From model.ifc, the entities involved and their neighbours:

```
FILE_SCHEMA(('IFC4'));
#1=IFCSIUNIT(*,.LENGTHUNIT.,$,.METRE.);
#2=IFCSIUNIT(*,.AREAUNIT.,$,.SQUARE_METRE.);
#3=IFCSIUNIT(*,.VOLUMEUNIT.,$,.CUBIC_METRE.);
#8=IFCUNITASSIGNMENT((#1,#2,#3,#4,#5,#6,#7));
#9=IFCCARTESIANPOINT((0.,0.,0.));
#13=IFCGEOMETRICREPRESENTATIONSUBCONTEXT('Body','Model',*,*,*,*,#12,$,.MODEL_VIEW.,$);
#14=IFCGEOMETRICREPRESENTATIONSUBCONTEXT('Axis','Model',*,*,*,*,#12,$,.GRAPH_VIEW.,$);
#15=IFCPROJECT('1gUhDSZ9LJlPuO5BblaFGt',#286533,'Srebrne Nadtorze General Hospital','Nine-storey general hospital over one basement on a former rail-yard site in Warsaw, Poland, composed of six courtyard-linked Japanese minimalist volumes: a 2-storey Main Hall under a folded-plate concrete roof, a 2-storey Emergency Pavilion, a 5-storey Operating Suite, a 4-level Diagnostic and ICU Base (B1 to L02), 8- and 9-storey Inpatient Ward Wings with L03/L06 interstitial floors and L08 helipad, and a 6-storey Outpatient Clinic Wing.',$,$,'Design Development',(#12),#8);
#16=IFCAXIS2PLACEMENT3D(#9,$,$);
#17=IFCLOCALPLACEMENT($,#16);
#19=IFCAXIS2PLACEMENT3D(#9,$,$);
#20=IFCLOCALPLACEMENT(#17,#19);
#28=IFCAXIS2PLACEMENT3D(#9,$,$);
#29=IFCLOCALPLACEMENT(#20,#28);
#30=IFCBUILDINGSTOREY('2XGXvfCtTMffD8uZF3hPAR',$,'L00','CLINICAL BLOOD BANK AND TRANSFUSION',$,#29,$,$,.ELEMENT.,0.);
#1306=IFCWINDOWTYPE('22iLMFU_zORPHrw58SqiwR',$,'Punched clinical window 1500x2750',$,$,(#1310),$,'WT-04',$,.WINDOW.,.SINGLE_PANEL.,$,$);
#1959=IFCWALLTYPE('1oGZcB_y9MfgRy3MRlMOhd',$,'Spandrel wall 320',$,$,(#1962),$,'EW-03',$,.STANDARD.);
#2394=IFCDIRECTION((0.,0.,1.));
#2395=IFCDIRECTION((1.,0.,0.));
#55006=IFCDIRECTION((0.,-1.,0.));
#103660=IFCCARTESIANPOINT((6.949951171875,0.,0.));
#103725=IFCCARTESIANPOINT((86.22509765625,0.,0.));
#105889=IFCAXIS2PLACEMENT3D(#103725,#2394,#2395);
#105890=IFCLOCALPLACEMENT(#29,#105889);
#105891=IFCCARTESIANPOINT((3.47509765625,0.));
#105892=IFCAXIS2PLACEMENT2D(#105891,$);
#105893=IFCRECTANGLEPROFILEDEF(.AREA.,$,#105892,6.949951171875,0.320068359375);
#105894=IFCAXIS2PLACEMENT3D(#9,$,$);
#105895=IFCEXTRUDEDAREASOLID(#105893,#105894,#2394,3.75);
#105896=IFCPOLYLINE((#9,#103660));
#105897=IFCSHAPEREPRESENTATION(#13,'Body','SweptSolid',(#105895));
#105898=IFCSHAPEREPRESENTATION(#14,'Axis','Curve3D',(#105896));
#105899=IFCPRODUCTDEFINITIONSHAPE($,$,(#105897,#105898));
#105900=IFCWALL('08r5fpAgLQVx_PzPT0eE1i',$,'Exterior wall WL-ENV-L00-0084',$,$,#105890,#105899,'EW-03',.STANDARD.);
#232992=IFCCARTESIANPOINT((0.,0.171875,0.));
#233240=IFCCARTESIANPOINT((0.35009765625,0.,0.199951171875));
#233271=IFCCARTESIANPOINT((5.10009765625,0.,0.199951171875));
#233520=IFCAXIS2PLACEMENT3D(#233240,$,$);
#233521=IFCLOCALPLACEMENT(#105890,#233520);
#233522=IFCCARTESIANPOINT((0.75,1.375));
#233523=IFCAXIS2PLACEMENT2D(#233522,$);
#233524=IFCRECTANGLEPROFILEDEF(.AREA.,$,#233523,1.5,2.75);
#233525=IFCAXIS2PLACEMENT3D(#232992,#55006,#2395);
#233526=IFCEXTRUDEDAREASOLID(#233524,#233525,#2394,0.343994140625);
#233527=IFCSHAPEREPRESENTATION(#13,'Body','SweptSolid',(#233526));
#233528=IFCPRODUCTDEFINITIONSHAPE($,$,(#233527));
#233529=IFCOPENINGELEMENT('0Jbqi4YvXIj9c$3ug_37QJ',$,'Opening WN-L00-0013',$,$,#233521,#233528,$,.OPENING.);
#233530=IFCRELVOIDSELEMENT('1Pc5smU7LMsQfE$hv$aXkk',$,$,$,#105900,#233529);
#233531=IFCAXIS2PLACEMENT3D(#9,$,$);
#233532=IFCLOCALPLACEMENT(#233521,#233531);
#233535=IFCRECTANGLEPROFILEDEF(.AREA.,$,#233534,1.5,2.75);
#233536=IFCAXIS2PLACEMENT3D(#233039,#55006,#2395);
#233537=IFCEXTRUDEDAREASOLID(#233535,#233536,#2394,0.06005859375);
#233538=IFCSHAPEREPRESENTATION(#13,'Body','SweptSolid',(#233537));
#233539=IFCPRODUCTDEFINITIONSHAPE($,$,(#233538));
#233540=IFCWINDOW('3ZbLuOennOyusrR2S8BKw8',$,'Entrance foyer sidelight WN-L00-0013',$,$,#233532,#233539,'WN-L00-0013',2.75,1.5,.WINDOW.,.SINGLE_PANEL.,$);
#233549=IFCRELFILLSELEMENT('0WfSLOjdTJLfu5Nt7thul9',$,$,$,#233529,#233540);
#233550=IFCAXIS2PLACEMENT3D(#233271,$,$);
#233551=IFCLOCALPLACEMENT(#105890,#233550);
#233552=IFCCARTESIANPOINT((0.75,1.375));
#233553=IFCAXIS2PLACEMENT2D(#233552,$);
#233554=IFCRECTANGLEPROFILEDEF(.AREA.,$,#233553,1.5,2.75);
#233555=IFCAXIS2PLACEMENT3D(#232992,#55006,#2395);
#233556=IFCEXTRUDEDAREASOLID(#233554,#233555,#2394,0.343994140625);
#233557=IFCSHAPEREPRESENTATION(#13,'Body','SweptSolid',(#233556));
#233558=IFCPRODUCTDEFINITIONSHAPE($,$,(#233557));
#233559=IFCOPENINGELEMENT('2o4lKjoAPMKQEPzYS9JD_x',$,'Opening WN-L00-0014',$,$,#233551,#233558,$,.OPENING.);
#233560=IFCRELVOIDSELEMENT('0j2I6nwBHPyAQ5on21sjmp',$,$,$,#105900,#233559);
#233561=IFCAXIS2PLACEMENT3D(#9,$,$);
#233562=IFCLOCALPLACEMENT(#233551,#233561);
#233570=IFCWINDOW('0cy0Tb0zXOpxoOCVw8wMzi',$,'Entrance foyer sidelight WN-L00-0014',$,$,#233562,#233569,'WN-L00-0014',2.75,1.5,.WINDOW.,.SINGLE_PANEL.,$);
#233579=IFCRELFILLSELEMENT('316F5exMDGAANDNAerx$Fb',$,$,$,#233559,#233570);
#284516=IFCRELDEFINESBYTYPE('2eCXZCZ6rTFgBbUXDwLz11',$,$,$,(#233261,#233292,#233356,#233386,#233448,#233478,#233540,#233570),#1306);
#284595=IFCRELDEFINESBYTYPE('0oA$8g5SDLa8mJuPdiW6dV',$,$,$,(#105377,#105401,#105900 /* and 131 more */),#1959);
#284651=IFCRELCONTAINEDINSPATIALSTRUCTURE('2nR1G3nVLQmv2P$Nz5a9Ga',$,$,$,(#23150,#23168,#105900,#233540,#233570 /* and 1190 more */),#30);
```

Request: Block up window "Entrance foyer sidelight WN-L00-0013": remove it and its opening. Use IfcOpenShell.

```python
import ifcopenshell
import ifcopenshell.api.feature
import ifcopenshell.api.root
import ifcopenshell.geom
import ifcopenshell.util.shape

model = ifcopenshell.open("model.ifc")
settings = ifcopenshell.geom.settings()


def volume(element):
    """Net volume in cubic metres, openings subtracted."""
    shape = ifcopenshell.geom.create_shape(settings, element)
    return ifcopenshell.util.shape.get_volume(shape.geometry)


window = model.by_guid("3ZbLuOennOyusrR2S8BKw8")
opening = window.FillsVoids[0].RelatingOpeningElement
wall = opening.VoidsElements[0].RelatingBuildingElement
before = volume(wall)

ifcopenshell.api.root.remove_product(model, product=window)
ifcopenshell.api.feature.remove_feature(model, feature=opening)

after = volume(wall)

print(f"wall volume {before:.3f} -> {after:.3f} m3")

model.write("model_v2.ifc")
```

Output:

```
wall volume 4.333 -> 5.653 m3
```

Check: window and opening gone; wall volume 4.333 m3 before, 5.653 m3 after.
